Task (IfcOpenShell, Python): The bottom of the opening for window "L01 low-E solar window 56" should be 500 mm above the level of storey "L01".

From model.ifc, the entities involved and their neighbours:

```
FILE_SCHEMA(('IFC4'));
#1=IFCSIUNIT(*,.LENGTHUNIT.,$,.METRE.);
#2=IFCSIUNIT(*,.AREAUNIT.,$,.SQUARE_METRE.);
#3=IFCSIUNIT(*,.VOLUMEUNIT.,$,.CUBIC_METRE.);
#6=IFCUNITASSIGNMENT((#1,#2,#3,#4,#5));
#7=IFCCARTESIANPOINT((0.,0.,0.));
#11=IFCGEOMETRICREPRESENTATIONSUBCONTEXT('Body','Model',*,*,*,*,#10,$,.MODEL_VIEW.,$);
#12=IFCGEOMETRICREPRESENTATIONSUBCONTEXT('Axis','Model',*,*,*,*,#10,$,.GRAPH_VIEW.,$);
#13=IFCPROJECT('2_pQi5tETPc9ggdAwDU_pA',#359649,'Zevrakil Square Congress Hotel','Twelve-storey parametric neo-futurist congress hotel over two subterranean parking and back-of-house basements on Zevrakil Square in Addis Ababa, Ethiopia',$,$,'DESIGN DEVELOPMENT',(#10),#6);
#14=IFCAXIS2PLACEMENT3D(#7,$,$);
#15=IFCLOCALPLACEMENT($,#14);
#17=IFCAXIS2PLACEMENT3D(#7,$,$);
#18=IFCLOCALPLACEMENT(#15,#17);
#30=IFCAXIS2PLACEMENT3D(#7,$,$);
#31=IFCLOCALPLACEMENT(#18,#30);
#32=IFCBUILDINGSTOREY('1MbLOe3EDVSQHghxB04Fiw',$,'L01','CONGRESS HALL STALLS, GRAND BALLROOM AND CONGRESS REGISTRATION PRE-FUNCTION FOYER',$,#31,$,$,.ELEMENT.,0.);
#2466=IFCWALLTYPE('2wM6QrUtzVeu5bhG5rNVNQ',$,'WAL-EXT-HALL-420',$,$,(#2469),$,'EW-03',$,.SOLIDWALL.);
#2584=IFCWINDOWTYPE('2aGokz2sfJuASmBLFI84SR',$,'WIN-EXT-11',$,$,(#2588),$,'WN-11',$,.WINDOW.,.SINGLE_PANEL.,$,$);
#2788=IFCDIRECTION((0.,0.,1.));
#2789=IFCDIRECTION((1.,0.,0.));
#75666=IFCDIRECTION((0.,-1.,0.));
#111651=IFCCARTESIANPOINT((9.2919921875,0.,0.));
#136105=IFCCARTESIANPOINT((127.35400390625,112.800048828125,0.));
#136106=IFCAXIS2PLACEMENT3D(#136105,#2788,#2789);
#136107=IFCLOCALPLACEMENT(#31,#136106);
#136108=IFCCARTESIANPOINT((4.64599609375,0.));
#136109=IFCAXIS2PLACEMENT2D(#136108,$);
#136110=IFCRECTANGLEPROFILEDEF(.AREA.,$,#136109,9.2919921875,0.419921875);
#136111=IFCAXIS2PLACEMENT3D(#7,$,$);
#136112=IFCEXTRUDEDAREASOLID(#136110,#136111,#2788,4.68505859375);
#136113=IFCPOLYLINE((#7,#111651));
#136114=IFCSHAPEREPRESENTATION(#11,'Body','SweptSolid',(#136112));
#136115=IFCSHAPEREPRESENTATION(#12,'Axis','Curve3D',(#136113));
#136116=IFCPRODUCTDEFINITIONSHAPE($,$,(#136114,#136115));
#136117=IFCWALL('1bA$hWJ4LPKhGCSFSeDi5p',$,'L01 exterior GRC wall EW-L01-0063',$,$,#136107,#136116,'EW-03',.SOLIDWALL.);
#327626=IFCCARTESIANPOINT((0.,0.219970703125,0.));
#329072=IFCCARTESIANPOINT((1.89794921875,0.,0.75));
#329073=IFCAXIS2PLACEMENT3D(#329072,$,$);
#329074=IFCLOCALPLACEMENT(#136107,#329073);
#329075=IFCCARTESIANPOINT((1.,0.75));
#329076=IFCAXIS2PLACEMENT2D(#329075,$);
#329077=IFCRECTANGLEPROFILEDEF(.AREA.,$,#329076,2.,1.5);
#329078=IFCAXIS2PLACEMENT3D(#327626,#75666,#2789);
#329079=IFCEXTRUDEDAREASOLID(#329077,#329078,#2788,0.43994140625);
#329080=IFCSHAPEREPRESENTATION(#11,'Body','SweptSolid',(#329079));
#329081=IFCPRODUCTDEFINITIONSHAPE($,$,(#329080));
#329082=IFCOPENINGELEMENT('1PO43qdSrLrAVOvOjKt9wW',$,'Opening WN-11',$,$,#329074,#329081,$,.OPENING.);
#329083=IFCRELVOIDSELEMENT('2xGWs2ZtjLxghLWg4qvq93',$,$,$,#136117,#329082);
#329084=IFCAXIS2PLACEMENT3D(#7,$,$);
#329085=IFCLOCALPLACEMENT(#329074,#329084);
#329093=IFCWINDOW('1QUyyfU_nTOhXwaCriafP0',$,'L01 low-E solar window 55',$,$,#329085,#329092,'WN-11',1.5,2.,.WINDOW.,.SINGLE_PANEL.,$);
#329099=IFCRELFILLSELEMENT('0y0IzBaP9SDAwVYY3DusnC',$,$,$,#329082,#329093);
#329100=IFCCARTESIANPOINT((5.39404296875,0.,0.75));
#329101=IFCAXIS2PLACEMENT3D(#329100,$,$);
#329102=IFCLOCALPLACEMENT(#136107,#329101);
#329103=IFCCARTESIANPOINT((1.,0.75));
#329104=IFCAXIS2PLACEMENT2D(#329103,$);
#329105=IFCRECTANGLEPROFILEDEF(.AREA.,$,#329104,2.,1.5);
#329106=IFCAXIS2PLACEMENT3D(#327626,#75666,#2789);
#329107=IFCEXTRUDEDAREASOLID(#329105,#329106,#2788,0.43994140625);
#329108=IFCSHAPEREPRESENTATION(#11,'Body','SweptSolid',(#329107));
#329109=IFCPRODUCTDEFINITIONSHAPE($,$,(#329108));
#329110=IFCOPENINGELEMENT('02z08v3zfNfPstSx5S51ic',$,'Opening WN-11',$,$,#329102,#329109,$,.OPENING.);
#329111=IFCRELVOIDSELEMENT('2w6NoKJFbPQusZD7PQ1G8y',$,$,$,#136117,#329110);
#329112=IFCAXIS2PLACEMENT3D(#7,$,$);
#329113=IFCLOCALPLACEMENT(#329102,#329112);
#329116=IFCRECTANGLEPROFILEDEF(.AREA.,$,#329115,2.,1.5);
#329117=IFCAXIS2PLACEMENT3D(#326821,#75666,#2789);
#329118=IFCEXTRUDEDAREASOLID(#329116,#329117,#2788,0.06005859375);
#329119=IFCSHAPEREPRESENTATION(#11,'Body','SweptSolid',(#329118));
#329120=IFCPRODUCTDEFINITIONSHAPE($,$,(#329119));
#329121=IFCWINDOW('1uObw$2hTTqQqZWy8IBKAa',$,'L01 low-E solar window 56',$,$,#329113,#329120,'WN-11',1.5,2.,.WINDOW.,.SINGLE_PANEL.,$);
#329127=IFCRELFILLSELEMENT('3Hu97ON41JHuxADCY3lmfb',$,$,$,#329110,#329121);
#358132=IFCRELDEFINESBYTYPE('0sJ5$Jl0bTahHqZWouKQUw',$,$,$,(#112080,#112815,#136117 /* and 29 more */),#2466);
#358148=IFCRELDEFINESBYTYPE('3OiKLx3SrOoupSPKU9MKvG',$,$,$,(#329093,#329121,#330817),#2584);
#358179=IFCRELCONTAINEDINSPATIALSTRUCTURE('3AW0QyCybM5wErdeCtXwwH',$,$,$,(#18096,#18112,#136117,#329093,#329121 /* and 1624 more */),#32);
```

```python
import numpy as np
import ifcopenshell
import ifcopenshell.api.geometry
import ifcopenshell.geom
import ifcopenshell.util.element
import ifcopenshell.util.placement
import ifcopenshell.util.shape
import ifcopenshell.util.unit

model = ifcopenshell.open("model.ifc")
unit_scale = ifcopenshell.util.unit.calculate_unit_scale(model)

window = model.by_guid("1uObw$2hTTqQqZWy8IBKAa")
opening = window.FillsVoids[0].RelatingOpeningElement
storey = ifcopenshell.util.element.get_container(window, ifc_class="IfcBuildingStorey")
level = ifcopenshell.util.placement.get_local_placement(storey.ObjectPlacement)[2, 3]

# The opening's origin need not be at the sill, so measure its lowest point.
shape = ifcopenshell.geom.create_shape(ifcopenshell.geom.settings(), opening)
bottom = ifcopenshell.util.shape.get_shape_bottom_elevation(shape, shape.geometry) / unit_scale
dz = level + 0.5 - bottom

shift = np.array([0.0, 0.0, dz])
# The window is placed relative to its opening, so it follows when the opening moves.
matrix = ifcopenshell.util.placement.get_local_placement(opening.ObjectPlacement)
matrix[:3, 3] += shift
ifcopenshell.api.geometry.edit_object_placement(
    model, product=opening, matrix=matrix, is_si=False, should_transform_children=True
)

print(f"moved by {dz * unit_scale:+.3f} m")

model.write("model_v2.ifc")
```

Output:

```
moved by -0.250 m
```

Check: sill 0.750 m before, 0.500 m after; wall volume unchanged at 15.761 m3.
